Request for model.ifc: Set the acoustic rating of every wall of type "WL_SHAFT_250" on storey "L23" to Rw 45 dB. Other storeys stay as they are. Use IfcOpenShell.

First a look at what the model holds.

```python
import ifcopenshell
import ifcopenshell.util.element

model = ifcopenshell.open("model.ifc")
print(model.schema)
storey = next(s for s in model.by_type("IfcBuildingStorey") if s.Name == "L23")
walls = [e for e in ifcopenshell.util.element.get_decomposition(storey) if e.is_a("IfcWall")]
seen = {}
for e in walls:
    element_type = ifcopenshell.util.element.get_type(e)
    key = (element_type.Name if element_type != e and element_type else None, ifcopenshell.util.element.get_pset(e, "Pset_WallCommon", "AcousticRating"))
    seen[key] = seen.get(key, 0) + 1
for (name, value), count in sorted(seen.items(), key=str):
    print(count, "x", name, "|", value)
```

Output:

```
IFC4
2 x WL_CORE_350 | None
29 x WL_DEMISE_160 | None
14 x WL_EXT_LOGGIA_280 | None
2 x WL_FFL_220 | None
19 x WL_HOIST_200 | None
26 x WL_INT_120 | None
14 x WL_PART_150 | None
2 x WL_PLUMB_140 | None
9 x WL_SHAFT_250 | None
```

```python
import ifcopenshell
import ifcopenshell.api.pset
import ifcopenshell.util.element

model = ifcopenshell.open("model.ifc")

storey = next(s for s in model.by_type("IfcBuildingStorey") if s.Name == "L23")
walls = [e for e in ifcopenshell.util.element.get_decomposition(storey) if e.is_a("IfcWall")]

count = 0
for e in walls:
    element_type = ifcopenshell.util.element.get_type(e)
    if element_type in (None, e) or element_type.Name != "WL_SHAFT_250":
        continue
    found = ifcopenshell.util.element.get_pset(e, "Pset_WallCommon", should_inherit=False)
    if found:
        pset = model.by_id(found["id"])
        if len(ifcopenshell.util.element.get_elements_by_pset(pset)) > 1:
            pset = ifcopenshell.api.pset.unshare_pset(model, products=[e], pset=pset)[0]
    else:
        pset = ifcopenshell.api.pset.add_pset(model, product=e, name="Pset_WallCommon")
    ifcopenshell.api.pset.edit_pset(model, pset=pset, properties={"AcousticRating": "Rw 45 dB"})
    count += 1

print(count, "walls updated")

model.write("model_updated.ifc")
```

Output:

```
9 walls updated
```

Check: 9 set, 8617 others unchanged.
